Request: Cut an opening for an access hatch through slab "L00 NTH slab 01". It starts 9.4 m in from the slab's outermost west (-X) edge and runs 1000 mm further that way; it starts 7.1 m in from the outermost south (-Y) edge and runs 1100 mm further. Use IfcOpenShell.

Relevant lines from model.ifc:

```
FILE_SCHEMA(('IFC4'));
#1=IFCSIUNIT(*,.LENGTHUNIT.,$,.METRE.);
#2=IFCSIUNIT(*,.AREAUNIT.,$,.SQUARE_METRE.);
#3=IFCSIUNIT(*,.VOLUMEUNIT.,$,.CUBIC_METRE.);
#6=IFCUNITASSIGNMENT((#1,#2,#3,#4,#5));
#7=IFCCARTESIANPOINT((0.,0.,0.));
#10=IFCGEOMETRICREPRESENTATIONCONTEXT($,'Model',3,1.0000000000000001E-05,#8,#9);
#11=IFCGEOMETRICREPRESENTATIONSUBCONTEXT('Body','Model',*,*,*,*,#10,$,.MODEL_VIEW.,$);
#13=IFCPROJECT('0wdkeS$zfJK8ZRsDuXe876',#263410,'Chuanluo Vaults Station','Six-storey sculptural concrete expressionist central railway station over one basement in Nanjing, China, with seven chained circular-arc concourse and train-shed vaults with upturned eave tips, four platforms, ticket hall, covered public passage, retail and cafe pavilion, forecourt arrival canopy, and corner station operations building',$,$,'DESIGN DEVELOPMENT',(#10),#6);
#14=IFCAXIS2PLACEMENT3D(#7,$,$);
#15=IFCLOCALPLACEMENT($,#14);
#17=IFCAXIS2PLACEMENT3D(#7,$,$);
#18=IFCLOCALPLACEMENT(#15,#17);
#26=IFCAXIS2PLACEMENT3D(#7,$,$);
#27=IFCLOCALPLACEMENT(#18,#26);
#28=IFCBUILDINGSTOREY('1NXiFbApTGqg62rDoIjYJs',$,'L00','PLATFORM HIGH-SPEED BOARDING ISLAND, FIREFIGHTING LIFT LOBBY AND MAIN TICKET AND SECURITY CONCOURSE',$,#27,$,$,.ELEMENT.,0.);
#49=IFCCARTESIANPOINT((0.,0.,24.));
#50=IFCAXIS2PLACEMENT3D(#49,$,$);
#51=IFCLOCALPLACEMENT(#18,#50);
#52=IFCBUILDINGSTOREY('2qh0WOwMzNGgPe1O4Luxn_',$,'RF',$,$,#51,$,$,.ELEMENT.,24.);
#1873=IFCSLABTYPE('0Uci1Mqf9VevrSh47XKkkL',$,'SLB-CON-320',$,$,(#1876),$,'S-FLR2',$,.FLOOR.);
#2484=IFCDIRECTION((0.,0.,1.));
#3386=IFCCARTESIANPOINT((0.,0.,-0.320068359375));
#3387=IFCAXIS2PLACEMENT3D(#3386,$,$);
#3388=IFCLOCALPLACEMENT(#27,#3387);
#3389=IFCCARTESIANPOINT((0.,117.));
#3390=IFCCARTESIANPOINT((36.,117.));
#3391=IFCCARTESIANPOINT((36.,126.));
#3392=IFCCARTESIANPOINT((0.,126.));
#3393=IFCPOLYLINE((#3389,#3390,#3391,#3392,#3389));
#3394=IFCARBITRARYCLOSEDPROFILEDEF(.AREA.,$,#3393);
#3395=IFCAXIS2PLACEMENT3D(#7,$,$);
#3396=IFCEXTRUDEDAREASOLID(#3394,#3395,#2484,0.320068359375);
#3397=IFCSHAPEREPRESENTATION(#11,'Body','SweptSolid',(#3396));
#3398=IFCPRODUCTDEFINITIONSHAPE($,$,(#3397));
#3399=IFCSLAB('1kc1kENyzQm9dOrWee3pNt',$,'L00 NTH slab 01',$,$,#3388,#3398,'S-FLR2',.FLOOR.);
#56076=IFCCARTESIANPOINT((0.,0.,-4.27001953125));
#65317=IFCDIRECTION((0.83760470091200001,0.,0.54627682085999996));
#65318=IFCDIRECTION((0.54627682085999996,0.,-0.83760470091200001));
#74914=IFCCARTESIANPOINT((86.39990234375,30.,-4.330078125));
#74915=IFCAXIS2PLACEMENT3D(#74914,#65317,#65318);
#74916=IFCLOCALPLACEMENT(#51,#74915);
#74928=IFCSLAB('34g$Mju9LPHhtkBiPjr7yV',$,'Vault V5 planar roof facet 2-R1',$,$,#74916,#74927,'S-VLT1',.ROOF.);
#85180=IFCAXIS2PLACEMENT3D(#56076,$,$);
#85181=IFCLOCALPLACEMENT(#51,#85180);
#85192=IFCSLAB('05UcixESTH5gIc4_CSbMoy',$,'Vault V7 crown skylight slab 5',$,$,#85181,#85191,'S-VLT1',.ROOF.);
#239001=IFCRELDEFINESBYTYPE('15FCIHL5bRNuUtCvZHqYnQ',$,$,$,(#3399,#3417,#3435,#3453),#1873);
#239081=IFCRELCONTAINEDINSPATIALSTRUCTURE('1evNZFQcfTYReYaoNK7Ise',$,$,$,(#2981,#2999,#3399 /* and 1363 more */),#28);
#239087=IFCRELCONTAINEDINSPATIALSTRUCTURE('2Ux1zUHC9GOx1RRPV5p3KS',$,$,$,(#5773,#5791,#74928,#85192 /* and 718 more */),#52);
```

```python
import numpy as np
import ifcopenshell
import ifcopenshell.api.feature
import ifcopenshell.api.geometry
import ifcopenshell.api.root
import ifcopenshell.geom
import ifcopenshell.util.placement
import ifcopenshell.util.representation
import ifcopenshell.util.shape
import ifcopenshell.util.unit

model = ifcopenshell.open("model.ifc")
unit_scale = ifcopenshell.util.unit.calculate_unit_scale(model)
settings = ifcopenshell.geom.settings()


def volume(element):
    """Net volume in cubic metres, openings subtracted."""
    shape = ifcopenshell.geom.create_shape(settings, element)
    return ifcopenshell.util.shape.get_volume(shape.geometry)


slab = model.by_id(3399)
before = volume(slab)

# Extent in the slab's own axes, in metres. The edges named are its -X and -Y sides.
slab_shape = ifcopenshell.geom.create_shape(settings, slab)
vertices = ifcopenshell.util.shape.get_vertices(slab_shape.geometry)
x_min, y_min, bottom = vertices.min(axis=0)
top = vertices[:, 2].max()

opening = ifcopenshell.api.root.create_entity(model, ifc_class="IfcOpeningElement", name="Access hatch opening", predefined_type="OPENING")
context = ifcopenshell.util.representation.get_context(model, "Model", "Body", "MODEL_VIEW")
width, depth = 1, 1.1
outline = [(0.0, 0.0), (width, 0.0), (width, depth), (0.0, depth), (0.0, 0.0)]
# Overshoot both faces by 50 mm so the cut is clean.
shape = ifcopenshell.api.geometry.add_slab_representation(
    model, context=context, depth=top - bottom + 0.1, polyline=outline
)
ifcopenshell.api.geometry.assign_representation(model, product=opening, representation=shape)

matrix = ifcopenshell.util.placement.get_local_placement(slab.ObjectPlacement)
matrix[:, 3] = matrix @ np.append(np.array([x_min + 9.4, y_min + 7.1, bottom - 0.05]) / unit_scale, 1.0)
ifcopenshell.api.geometry.edit_object_placement(model, product=opening, matrix=matrix, is_si=False)
ifcopenshell.api.feature.add_feature(model, feature=opening, element=slab)

after = volume(slab)

print(f"slab volume {before:.3f} -> {after:.3f} m3")

model.write("model_v2.ifc")
```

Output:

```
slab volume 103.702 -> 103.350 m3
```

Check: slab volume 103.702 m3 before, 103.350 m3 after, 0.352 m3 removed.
